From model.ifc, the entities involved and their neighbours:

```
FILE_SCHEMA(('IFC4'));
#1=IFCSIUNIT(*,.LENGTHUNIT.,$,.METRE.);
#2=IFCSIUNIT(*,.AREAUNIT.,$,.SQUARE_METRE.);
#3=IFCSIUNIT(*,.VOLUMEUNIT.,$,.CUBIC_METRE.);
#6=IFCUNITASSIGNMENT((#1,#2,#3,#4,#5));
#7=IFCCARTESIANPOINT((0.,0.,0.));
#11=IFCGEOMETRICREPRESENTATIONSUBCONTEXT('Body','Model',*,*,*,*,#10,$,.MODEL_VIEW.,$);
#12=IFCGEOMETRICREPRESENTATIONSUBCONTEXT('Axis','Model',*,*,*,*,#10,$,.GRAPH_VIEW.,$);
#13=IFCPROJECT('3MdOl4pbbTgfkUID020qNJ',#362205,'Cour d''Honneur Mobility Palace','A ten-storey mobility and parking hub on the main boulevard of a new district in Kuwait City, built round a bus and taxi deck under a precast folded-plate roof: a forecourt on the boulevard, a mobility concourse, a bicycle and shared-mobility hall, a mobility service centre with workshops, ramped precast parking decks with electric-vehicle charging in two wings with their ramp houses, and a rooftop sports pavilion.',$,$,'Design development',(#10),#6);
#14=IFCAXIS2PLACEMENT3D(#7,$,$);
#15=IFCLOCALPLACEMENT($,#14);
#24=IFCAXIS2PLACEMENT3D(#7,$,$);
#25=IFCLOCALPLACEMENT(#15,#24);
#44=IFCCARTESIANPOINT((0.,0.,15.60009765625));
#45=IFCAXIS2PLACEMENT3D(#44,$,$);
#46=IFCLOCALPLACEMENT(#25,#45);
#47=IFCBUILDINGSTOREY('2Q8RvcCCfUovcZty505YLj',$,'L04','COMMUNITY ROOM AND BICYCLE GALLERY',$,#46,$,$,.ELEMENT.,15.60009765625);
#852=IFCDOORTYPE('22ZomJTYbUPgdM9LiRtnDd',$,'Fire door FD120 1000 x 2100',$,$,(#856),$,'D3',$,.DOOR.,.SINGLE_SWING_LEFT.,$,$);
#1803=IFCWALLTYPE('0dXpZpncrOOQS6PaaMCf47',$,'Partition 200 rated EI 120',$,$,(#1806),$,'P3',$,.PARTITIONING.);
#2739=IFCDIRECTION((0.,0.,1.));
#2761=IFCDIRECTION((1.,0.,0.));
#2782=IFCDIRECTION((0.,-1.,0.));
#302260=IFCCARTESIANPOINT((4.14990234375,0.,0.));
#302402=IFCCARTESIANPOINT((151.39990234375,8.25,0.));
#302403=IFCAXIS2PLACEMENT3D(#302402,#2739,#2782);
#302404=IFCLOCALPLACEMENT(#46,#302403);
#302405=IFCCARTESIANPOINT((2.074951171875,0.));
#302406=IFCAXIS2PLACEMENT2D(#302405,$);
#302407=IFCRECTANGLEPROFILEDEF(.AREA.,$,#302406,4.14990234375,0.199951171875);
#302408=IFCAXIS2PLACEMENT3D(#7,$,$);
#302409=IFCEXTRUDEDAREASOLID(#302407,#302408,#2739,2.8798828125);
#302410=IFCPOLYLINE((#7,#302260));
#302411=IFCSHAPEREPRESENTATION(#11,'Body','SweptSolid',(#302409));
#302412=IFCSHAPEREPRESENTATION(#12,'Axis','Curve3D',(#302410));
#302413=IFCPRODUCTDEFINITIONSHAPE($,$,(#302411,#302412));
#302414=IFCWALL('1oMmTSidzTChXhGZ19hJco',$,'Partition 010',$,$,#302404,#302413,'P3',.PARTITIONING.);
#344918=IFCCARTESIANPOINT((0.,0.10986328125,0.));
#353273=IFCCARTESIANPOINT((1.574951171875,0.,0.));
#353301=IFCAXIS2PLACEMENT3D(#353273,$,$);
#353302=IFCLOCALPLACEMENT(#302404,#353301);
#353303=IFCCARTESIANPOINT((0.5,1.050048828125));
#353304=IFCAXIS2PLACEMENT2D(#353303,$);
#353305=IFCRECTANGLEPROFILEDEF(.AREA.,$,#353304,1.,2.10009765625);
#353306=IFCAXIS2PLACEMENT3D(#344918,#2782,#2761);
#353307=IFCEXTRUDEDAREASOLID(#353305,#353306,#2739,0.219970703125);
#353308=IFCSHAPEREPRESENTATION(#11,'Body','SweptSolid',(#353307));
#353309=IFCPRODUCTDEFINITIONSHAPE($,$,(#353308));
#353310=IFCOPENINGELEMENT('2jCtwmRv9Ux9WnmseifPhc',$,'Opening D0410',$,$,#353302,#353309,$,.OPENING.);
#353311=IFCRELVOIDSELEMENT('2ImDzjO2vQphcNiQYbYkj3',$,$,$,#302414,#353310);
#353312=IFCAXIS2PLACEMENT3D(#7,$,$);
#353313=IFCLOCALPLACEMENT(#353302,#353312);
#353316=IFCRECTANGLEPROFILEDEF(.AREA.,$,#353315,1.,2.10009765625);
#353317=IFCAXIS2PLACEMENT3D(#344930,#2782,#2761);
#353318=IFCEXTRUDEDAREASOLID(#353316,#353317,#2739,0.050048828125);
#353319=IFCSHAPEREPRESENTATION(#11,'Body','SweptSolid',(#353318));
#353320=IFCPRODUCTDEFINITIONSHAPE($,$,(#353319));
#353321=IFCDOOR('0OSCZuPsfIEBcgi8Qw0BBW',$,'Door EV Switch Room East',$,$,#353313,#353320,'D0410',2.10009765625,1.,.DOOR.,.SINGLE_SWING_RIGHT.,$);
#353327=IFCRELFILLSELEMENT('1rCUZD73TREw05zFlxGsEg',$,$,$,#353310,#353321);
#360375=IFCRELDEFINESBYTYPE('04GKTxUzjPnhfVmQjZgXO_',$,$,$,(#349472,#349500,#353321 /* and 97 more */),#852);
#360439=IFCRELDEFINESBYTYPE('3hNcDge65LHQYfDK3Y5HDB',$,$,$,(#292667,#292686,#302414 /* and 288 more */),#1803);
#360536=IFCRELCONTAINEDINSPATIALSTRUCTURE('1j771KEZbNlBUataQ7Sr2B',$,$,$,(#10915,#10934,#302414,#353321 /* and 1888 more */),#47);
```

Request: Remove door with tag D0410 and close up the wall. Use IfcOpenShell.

```python
import ifcopenshell
import ifcopenshell.api.feature
import ifcopenshell.api.root
import ifcopenshell.geom
import ifcopenshell.util.shape

model = ifcopenshell.open("model.ifc")
settings = ifcopenshell.geom.settings()


def volume(element):
    """Net volume in cubic metres, openings subtracted."""
    shape = ifcopenshell.geom.create_shape(settings, element)
    return ifcopenshell.util.shape.get_volume(shape.geometry)


door = model.by_guid("0OSCZuPsfIEBcgi8Qw0BBW")
opening = door.FillsVoids[0].RelatingOpeningElement
wall = opening.VoidsElements[0].RelatingBuildingElement
before = volume(wall)

ifcopenshell.api.root.remove_product(model, product=door)
ifcopenshell.api.feature.remove_feature(model, feature=opening)

after = volume(wall)

print(f"wall volume {before:.3f} -> {after:.3f} m3")

model.write("model_v2.ifc")
```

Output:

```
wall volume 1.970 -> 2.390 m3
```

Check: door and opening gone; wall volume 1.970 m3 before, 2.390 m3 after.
